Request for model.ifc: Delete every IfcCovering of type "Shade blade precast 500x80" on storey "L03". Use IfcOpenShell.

First a look at what the model holds.

```python
import ifcopenshell
import ifcopenshell.util.element

model = ifcopenshell.open("model.ifc")
print(model.schema)
storey = next(s for s in model.by_type("IfcBuildingStorey") if s.Name == "L03")
coverings = [e for e in ifcopenshell.util.element.get_decomposition(storey) if e.is_a("IfcCovering")]
seen = {}
for e in coverings:
    element_type = ifcopenshell.util.element.get_type(e)
    name = element_type.Name if element_type not in (None, e) else None
    seen[name] = seen.get(name, 0) + 1
for name, count in sorted(seen.items(), key=str):
    print(count, "x", name)
```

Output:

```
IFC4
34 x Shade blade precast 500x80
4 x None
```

```python
import ifcopenshell
import ifcopenshell.api.root
import ifcopenshell.util.element

model = ifcopenshell.open("model.ifc")

storey = next(s for s in model.by_type("IfcBuildingStorey") if s.Name == "L03")
coverings = [e for e in ifcopenshell.util.element.get_decomposition(storey) if e.is_a("IfcCovering")]
targets = [e for e in coverings if (t := ifcopenshell.util.element.get_type(e)) not in (None, e) and t.Name == "Shade blade precast 500x80"]

for e in targets:
    ifcopenshell.api.root.remove_product(model, product=e)
print(len(targets), "removed")

model.write("model-out.ifc")
```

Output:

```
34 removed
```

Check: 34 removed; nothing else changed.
